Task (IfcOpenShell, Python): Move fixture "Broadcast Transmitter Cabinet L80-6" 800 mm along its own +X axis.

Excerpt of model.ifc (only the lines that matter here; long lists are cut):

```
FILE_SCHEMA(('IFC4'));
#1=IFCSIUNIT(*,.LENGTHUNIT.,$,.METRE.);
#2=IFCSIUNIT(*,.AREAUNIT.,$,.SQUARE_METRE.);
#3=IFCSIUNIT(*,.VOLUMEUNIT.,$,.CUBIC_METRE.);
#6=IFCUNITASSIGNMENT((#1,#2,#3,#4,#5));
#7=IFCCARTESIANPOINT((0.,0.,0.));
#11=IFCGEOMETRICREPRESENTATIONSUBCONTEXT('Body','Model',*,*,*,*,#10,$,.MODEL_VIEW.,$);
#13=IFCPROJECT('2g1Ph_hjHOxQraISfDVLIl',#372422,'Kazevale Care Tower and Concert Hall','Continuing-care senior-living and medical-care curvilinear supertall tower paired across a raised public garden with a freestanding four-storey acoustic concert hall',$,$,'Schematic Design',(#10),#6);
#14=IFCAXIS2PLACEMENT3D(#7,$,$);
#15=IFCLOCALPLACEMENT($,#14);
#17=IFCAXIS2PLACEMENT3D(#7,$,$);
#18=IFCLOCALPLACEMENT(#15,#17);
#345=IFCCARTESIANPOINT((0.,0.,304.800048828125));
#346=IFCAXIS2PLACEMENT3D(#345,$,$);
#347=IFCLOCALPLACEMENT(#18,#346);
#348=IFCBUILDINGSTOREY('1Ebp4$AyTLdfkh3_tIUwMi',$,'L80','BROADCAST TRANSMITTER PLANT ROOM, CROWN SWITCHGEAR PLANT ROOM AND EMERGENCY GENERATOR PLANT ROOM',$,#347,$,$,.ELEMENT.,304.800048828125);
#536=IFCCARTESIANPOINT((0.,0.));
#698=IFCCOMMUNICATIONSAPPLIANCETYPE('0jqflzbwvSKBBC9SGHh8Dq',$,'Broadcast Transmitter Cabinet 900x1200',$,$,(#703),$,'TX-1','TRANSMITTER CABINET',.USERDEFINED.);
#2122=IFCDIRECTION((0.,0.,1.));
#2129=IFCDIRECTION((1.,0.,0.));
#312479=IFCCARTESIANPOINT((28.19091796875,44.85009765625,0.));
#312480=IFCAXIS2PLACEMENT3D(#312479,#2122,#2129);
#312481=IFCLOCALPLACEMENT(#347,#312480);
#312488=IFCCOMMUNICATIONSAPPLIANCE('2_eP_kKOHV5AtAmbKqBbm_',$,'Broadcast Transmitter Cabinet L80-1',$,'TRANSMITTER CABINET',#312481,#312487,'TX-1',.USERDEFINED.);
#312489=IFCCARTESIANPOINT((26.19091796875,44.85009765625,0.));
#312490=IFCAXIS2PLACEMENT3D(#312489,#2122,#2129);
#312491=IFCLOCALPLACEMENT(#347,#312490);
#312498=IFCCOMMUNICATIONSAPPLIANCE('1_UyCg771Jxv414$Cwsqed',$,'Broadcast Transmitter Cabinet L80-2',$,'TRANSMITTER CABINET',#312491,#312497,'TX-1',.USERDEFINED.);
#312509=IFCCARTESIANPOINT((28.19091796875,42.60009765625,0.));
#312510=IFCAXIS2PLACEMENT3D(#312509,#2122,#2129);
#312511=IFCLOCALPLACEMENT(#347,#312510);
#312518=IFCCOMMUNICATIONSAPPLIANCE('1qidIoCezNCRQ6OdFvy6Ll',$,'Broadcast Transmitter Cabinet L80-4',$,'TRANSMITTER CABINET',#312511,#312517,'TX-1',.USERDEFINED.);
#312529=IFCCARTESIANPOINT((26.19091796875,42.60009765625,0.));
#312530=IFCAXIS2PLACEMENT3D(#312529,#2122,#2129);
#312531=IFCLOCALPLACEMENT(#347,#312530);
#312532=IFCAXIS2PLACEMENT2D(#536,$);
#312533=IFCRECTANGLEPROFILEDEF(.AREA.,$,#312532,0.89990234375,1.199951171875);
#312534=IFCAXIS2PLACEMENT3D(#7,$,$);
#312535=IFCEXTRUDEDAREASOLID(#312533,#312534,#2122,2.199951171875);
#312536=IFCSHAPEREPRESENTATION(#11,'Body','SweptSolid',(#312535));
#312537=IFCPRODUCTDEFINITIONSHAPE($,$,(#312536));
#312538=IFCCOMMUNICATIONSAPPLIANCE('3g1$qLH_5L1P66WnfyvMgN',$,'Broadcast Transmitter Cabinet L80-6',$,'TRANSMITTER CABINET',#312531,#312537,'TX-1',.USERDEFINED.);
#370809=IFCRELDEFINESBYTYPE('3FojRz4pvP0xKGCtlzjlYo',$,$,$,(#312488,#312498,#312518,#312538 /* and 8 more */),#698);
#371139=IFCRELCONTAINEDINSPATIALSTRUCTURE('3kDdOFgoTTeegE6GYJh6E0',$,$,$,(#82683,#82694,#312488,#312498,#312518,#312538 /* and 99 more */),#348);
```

```python
import ifcopenshell
import ifcopenshell.api.geometry
import ifcopenshell.util.placement
import ifcopenshell.util.unit

model = ifcopenshell.open("model.ifc")
unit_scale = ifcopenshell.util.unit.calculate_unit_scale(model)

item = model.by_guid("3g1$qLH_5L1P66WnfyvMgN")
matrix = ifcopenshell.util.placement.get_local_placement(item.ObjectPlacement)
matrix[:3, 3] += matrix[:3, 0] * 0.8 / unit_scale
ifcopenshell.api.geometry.edit_object_placement(model, product=item, matrix=matrix, is_si=False)

print(ifcopenshell.util.placement.get_local_placement(item.ObjectPlacement).round(3) + 0.0)

model.write("model_rev.ifc")
```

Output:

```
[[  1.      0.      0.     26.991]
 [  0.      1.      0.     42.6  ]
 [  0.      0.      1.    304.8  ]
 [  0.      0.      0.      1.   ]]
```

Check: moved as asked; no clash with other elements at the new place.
